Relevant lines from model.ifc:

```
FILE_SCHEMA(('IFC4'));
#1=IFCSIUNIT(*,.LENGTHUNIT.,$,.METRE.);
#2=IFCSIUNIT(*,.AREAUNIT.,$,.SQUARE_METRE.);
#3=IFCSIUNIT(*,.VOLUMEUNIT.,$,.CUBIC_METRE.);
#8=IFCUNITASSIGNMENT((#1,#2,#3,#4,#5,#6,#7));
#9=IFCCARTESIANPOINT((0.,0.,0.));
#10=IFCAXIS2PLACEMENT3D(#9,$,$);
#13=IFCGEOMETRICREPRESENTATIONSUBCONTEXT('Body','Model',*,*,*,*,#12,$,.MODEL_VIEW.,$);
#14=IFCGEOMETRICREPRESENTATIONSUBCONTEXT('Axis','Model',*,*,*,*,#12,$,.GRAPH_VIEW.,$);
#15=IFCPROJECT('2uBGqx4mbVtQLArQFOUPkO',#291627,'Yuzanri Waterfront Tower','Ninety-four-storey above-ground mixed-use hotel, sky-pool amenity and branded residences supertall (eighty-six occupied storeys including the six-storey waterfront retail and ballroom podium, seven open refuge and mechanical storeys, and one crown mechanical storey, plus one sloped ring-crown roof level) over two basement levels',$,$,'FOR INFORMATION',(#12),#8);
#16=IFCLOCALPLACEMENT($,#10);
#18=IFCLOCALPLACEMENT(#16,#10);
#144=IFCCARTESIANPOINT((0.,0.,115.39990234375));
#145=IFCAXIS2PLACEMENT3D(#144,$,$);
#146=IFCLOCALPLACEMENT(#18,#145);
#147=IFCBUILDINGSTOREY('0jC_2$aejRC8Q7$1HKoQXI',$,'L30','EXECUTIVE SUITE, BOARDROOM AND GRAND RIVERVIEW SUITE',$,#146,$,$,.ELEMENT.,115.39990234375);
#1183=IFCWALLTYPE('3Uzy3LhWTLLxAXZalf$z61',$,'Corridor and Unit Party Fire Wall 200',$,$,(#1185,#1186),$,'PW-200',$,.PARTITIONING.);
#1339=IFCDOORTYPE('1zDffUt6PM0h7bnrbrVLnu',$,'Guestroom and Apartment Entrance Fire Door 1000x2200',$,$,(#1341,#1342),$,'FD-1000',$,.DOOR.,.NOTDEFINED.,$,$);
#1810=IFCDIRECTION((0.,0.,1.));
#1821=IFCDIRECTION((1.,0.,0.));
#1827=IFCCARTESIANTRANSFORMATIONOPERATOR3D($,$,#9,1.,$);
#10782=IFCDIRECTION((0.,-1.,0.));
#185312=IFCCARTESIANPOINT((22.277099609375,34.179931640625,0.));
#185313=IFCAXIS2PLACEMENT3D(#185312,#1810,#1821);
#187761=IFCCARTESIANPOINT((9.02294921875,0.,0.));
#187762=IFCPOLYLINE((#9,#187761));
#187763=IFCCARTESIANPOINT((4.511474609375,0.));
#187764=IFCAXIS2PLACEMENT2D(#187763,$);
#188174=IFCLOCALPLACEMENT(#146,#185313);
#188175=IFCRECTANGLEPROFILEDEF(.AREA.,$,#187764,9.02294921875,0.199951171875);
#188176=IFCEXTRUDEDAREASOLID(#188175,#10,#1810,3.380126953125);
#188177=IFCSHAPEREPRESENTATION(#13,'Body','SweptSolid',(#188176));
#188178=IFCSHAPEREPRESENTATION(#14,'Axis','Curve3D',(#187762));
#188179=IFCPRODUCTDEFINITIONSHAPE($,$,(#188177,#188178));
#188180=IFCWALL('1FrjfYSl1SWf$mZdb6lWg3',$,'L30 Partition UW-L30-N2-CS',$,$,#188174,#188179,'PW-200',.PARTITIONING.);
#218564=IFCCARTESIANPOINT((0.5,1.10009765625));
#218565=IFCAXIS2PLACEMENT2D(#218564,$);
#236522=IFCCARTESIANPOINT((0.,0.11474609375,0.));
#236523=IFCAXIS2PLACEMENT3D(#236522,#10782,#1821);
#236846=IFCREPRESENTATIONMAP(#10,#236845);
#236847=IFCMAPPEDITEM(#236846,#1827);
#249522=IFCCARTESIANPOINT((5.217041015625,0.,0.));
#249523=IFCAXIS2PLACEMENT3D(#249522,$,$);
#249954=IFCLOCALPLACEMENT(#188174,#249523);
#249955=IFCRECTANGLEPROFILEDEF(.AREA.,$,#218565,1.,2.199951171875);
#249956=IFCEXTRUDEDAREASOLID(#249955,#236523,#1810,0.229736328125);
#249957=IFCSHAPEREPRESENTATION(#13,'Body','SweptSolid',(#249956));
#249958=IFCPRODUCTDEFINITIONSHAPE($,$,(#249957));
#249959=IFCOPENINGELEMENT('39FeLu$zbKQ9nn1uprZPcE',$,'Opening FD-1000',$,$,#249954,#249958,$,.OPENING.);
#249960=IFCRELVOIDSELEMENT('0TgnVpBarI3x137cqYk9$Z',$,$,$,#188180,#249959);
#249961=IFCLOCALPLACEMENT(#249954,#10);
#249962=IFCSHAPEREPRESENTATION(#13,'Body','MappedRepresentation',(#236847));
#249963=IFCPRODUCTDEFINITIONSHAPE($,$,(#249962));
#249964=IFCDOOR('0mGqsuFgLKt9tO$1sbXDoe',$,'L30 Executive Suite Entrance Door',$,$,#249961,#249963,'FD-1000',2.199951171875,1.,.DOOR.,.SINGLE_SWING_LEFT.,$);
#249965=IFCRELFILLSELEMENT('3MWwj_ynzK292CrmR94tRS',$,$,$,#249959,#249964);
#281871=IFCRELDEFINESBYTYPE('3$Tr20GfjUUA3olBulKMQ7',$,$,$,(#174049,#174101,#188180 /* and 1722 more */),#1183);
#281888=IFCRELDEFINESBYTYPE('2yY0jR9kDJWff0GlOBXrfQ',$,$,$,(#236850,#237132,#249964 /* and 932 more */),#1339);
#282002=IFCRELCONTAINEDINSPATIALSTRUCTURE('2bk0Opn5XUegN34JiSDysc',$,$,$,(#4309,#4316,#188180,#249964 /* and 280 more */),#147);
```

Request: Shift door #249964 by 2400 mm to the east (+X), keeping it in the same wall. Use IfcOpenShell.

```python
import ifcopenshell
import ifcopenshell.api.geometry
import ifcopenshell.util.placement

model = ifcopenshell.open("model.ifc")

door = model.by_guid("0mGqsuFgLKt9tO$1sbXDoe")
opening = door.FillsVoids[0].RelatingOpeningElement
wall = opening.VoidsElements[0].RelatingBuildingElement

wall_matrix = ifcopenshell.util.placement.get_local_placement(wall.ObjectPlacement)
shift = wall_matrix[:3, 0] * 2.4
before = ifcopenshell.util.placement.get_local_placement(door.ObjectPlacement)[:3, 3].copy()

# The door is placed relative to its opening, so it follows when the opening moves.
matrix = ifcopenshell.util.placement.get_local_placement(opening.ObjectPlacement)
matrix[:3, 3] += shift
ifcopenshell.api.geometry.edit_object_placement(
    model, product=opening, matrix=matrix, is_si=False, should_transform_children=True
)

after = ifcopenshell.util.placement.get_local_placement(door.ObjectPlacement)[:3, 3]
print("door moved by", (after - before).round(3) + 0.0)

model.write("model_v2.ifc")
```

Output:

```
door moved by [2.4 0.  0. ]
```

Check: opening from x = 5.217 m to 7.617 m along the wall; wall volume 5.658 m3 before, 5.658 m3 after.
